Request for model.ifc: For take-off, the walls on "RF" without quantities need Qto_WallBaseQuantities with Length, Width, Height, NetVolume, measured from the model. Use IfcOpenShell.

First a look at what the model holds.

```python
import ifcopenshell
import ifcopenshell.util.element
import ifcopenshell.util.unit

model = ifcopenshell.open("model.ifc")
print(model.schema)
for unit_type in ("LENGTHUNIT", "AREAUNIT", "VOLUMEUNIT"):
    print(unit_type, ifcopenshell.util.unit.calculate_unit_scale(model, unit_type))
storey = next(s for s in model.by_type("IfcBuildingStorey") if s.Name == "RF")
walls = [e for e in ifcopenshell.util.element.get_decomposition(storey) if e.is_a("IfcWall")]
for e in sorted(walls, key=lambda e: e.id()):
    print(e.id(), e.is_a(), e.Name, list(ifcopenshell.util.element.get_psets(e, qtos_only=True)), sep=" | ")
```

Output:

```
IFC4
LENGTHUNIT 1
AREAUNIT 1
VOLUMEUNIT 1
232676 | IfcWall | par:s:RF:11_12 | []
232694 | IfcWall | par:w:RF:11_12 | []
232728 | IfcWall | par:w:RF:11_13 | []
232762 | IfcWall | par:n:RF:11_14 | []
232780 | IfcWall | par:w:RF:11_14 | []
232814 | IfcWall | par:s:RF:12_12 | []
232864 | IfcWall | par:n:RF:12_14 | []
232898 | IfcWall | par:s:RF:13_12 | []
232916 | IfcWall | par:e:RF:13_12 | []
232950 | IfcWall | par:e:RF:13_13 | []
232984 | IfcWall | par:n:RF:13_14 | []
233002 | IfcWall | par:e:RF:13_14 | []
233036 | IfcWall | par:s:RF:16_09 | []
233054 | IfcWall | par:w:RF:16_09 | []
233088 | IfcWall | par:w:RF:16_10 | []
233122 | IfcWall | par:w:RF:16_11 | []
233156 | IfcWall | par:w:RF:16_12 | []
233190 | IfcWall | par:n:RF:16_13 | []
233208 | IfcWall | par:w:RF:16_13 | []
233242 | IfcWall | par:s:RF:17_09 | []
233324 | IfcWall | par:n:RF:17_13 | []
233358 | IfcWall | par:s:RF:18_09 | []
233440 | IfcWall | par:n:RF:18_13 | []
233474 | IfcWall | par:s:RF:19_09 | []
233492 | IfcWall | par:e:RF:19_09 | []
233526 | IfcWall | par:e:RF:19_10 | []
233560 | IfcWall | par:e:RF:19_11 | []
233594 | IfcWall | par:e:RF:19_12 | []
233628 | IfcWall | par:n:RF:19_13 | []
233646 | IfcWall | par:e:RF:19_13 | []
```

```python
import ifcopenshell
import ifcopenshell.api.pset
import ifcopenshell.geom
import ifcopenshell.util.element
import ifcopenshell.util.shape
import ifcopenshell.util.unit

model = ifcopenshell.open("model.ifc")
unit_scale = ifcopenshell.util.unit.calculate_unit_scale(model)
volume_scale = ifcopenshell.util.unit.calculate_unit_scale(model, "VOLUMEUNIT")
settings = ifcopenshell.geom.settings()

storey = next(s for s in model.by_type("IfcBuildingStorey") if s.Name == "RF")
walls = [e for e in ifcopenshell.util.element.get_decomposition(storey) if e.is_a("IfcWall")]

for e in sorted(walls, key=lambda e: e.id()):
    if ifcopenshell.util.element.get_psets(e, qtos_only=True, should_inherit=False):
        continue
    # Geometry comes back in metres, in the element's own axes.
    shape = ifcopenshell.geom.create_shape(settings, e)
    values = {
        "Length": ifcopenshell.util.shape.get_x(shape.geometry) / unit_scale,
        "Width": ifcopenshell.util.shape.get_y(shape.geometry) / unit_scale,
        "Height": ifcopenshell.util.shape.get_z(shape.geometry) / unit_scale,
        "NetVolume": ifcopenshell.util.shape.get_volume(shape.geometry) / volume_scale,
    }
    qto = ifcopenshell.api.pset.add_qto(model, product=e, name="Qto_WallBaseQuantities")
    ifcopenshell.api.pset.edit_qto(model, qto=qto, properties=values)
    print(e.id(), {k: round(v, 3) for k, v in values.items()})

model.write("model-out.ifc")
```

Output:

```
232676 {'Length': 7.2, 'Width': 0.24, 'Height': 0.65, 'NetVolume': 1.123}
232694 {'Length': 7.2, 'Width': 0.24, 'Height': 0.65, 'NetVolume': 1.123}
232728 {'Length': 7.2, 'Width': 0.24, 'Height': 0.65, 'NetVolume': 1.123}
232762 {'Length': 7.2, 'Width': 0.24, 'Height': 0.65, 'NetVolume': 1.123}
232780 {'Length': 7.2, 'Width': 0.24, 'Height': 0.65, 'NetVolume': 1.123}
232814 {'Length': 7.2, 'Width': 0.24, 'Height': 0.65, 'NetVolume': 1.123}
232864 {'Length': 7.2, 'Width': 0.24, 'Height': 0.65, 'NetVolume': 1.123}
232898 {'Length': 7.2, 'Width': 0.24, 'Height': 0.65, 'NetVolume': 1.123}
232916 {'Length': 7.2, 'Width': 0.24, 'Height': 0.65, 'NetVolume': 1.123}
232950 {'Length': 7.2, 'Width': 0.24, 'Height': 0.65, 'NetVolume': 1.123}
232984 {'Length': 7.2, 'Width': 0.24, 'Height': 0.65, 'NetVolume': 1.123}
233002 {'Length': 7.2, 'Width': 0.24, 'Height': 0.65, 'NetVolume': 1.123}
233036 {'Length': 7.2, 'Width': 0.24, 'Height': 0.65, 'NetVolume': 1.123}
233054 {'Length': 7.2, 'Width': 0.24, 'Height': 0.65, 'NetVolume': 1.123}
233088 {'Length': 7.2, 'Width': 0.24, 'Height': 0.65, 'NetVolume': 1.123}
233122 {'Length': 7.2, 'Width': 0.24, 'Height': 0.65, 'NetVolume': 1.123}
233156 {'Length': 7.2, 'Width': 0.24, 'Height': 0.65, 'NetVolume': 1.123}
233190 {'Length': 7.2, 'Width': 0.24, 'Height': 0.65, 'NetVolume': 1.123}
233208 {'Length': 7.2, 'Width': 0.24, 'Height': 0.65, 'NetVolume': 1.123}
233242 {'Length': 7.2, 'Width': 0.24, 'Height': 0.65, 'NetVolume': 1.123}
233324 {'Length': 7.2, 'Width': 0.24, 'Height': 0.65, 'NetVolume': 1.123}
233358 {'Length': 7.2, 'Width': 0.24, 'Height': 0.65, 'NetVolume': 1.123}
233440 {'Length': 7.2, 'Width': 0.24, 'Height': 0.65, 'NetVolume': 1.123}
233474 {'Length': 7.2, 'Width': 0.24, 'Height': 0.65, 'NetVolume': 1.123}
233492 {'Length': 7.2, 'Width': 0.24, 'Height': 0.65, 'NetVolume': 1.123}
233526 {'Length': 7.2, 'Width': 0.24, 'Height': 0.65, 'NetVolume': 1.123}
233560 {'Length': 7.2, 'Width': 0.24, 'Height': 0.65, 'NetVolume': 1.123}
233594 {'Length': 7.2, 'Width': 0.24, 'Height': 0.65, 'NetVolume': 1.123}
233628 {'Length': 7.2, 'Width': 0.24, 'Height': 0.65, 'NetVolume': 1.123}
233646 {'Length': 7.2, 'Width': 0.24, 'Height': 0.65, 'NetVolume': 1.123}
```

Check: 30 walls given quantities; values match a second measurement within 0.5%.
